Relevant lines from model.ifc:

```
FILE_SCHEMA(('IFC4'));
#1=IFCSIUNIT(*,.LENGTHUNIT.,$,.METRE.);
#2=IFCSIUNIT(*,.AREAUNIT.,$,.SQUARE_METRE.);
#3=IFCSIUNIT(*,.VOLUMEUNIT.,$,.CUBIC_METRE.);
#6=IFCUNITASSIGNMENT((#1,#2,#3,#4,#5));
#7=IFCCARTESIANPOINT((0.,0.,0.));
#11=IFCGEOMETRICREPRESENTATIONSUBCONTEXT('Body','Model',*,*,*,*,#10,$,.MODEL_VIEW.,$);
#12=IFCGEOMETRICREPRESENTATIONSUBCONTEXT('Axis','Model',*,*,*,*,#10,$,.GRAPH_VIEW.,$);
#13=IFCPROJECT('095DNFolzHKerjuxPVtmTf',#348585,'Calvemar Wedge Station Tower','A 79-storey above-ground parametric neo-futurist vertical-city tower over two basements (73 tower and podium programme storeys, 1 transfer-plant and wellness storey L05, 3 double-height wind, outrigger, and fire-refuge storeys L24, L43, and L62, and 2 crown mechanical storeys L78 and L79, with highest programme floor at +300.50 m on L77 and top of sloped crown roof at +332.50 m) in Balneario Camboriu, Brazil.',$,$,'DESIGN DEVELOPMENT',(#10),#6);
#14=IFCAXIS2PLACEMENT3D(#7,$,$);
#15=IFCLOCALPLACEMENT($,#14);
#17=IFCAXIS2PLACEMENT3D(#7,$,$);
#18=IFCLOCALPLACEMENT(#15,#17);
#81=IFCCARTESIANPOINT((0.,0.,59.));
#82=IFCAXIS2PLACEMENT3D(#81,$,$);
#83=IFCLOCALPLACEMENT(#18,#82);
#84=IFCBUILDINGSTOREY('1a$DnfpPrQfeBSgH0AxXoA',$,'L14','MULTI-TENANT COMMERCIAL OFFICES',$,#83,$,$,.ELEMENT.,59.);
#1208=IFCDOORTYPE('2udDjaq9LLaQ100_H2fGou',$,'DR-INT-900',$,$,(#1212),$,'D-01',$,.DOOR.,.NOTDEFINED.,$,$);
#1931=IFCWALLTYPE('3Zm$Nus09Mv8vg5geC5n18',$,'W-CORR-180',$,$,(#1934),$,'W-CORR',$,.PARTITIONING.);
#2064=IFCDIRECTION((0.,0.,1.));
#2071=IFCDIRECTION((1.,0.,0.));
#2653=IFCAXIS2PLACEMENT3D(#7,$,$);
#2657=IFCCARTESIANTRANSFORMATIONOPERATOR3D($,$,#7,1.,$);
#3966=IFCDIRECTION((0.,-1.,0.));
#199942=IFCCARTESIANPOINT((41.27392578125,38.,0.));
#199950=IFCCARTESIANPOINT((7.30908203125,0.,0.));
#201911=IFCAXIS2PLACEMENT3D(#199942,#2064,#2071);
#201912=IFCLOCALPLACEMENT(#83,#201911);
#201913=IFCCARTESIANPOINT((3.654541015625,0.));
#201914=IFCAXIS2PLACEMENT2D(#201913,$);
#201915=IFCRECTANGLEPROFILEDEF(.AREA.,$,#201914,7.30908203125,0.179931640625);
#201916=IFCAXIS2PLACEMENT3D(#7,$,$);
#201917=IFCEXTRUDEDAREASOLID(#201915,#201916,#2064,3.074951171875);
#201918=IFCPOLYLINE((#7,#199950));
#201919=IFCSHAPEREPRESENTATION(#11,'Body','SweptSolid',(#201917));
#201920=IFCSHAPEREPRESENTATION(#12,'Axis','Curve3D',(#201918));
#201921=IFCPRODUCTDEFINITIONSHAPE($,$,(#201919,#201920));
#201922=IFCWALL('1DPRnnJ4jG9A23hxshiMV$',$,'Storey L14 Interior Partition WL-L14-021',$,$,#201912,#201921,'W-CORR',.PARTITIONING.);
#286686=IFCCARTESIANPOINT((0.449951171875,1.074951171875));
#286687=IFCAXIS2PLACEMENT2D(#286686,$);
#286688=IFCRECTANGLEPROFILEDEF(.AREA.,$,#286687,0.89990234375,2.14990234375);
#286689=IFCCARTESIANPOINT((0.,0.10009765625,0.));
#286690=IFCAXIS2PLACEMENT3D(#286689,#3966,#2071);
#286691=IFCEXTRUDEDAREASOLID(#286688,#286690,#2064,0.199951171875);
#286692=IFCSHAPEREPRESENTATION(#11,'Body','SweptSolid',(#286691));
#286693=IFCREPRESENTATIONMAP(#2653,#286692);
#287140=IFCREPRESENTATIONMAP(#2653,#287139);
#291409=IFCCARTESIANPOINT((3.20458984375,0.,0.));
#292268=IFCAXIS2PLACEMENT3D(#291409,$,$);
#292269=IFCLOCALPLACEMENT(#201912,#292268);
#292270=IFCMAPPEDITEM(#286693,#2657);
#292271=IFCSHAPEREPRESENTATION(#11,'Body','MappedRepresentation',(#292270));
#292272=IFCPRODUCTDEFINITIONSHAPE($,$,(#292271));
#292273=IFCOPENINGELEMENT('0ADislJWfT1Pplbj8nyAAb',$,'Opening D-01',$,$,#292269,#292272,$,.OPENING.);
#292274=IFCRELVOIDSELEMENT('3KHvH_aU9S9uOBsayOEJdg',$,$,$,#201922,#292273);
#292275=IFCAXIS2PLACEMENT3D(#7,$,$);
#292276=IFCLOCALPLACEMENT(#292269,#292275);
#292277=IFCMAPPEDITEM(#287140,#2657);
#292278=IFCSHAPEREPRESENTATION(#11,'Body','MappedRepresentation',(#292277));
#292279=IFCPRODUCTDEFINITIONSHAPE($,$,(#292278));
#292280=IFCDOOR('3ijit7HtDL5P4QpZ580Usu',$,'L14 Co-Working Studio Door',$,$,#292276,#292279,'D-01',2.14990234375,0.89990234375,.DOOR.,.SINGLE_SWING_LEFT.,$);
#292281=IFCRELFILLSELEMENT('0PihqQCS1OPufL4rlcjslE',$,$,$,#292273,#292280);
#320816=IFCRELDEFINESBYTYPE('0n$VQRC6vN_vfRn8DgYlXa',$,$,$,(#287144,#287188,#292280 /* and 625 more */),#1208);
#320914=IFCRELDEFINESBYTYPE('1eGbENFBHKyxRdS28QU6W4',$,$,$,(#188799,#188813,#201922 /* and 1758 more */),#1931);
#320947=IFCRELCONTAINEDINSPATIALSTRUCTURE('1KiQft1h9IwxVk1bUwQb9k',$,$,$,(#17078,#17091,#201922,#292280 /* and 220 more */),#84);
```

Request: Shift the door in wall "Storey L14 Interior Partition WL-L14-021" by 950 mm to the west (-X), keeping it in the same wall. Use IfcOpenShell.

```python
import ifcopenshell
import ifcopenshell.api.geometry
import ifcopenshell.util.placement

model = ifcopenshell.open("model.ifc")

door = model.by_guid("3ijit7HtDL5P4QpZ580Usu")
opening = door.FillsVoids[0].RelatingOpeningElement
wall = opening.VoidsElements[0].RelatingBuildingElement

wall_matrix = ifcopenshell.util.placement.get_local_placement(wall.ObjectPlacement)
shift = wall_matrix[:3, 0] * -0.95
before = ifcopenshell.util.placement.get_local_placement(door.ObjectPlacement)[:3, 3].copy()

# The door is placed relative to its opening, so it follows when the opening moves.
matrix = ifcopenshell.util.placement.get_local_placement(opening.ObjectPlacement)
matrix[:3, 3] += shift
ifcopenshell.api.geometry.edit_object_placement(
    model, product=opening, matrix=matrix, is_si=False, should_transform_children=True
)

after = ifcopenshell.util.placement.get_local_placement(door.ObjectPlacement)[:3, 3]
print("door moved by", (after - before).round(3) + 0.0)

model.write("model-out.ifc")
```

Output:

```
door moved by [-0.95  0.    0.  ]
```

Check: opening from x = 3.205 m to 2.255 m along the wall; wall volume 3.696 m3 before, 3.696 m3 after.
